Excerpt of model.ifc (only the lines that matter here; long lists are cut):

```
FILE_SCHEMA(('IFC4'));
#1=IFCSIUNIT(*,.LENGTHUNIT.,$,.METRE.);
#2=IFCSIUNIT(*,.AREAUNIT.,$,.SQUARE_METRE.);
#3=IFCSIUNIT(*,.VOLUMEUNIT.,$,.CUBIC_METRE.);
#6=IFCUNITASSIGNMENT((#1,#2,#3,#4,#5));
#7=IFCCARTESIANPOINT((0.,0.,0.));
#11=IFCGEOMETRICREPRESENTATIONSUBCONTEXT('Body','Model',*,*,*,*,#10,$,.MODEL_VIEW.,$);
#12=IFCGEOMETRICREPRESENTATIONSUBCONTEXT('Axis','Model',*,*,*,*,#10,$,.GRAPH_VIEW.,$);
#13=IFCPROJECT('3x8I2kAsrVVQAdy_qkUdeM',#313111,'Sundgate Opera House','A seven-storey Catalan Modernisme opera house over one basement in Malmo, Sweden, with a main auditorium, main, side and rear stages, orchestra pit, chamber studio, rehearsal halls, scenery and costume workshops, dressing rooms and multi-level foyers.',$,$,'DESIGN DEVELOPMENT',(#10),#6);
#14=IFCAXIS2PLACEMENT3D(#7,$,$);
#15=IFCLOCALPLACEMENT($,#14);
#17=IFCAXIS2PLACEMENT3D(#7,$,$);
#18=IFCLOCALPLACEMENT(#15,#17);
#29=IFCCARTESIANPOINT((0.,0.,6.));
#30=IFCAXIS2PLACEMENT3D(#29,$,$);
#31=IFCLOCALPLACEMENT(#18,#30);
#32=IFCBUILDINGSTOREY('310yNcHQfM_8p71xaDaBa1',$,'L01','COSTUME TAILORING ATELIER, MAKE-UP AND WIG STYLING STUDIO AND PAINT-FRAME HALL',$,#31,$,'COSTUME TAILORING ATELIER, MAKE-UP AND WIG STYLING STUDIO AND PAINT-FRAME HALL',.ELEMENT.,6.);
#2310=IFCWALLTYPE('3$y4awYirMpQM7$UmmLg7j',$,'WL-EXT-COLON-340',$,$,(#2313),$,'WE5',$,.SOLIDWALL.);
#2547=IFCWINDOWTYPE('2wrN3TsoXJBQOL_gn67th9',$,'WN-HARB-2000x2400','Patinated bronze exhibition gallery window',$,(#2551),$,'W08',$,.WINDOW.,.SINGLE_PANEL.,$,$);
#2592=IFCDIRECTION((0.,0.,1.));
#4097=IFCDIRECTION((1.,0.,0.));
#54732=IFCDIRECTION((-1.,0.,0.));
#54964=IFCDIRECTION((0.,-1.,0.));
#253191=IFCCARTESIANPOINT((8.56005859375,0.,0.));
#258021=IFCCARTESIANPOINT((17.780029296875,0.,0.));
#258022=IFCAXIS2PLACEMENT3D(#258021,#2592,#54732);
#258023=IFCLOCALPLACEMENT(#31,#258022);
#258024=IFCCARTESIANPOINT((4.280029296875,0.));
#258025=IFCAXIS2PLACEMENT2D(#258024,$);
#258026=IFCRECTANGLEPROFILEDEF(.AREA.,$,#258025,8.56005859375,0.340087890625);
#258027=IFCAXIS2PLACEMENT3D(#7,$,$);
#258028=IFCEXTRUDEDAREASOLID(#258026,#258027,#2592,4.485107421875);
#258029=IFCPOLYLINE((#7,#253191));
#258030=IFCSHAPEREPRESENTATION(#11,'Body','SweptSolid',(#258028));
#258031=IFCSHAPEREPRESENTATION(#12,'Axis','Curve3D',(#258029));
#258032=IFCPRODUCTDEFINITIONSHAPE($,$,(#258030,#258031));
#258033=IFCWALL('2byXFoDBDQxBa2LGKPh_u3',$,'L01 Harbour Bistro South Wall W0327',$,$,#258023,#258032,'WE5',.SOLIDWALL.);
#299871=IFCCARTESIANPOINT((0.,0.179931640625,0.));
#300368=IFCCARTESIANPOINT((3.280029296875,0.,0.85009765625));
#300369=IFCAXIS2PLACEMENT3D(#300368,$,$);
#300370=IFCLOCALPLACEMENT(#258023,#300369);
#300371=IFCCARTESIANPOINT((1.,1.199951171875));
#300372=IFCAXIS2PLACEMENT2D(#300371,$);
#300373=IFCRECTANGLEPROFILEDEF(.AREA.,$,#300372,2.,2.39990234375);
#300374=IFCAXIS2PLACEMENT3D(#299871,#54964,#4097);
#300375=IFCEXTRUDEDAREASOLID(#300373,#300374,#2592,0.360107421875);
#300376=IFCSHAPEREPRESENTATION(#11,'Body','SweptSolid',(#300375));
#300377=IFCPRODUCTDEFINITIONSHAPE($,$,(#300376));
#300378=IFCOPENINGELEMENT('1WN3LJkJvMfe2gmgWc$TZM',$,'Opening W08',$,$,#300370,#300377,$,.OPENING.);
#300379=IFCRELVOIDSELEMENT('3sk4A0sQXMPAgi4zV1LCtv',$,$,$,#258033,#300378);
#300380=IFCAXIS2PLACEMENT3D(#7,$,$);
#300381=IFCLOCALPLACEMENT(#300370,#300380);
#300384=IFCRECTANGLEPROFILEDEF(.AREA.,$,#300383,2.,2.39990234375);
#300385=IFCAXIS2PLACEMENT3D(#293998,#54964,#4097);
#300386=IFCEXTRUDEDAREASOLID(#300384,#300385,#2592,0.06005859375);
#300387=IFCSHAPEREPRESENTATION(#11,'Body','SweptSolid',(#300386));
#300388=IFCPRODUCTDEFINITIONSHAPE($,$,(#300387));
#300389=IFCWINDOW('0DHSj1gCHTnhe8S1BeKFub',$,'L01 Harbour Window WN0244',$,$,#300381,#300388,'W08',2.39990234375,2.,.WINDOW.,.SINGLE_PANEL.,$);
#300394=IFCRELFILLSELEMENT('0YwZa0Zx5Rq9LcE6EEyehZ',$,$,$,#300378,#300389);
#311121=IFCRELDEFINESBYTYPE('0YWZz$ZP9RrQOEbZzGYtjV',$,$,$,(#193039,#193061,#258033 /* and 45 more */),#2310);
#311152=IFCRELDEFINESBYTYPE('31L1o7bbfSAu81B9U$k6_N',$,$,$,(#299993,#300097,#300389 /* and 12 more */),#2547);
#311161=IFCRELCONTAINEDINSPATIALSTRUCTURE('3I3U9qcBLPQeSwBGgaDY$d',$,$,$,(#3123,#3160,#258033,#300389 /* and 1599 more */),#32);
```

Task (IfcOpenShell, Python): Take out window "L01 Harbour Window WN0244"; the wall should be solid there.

```python
import ifcopenshell
import ifcopenshell.api.feature
import ifcopenshell.api.root
import ifcopenshell.geom
import ifcopenshell.util.shape

model = ifcopenshell.open("model.ifc")
settings = ifcopenshell.geom.settings()


def volume(element):
    """Net volume in cubic metres, openings subtracted."""
    shape = ifcopenshell.geom.create_shape(settings, element)
    return ifcopenshell.util.shape.get_volume(shape.geometry)


window = model.by_id(300389)
opening = window.FillsVoids[0].RelatingOpeningElement
wall = opening.VoidsElements[0].RelatingBuildingElement
before = volume(wall)

ifcopenshell.api.root.remove_product(model, product=window)
ifcopenshell.api.feature.remove_feature(model, feature=opening)

after = volume(wall)

print(f"wall volume {before:.3f} -> {after:.3f} m3")

model.write("model_v2.ifc")
```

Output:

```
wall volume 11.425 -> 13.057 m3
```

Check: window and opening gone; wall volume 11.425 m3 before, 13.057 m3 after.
